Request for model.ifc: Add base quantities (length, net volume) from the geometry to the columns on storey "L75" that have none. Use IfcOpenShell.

First a look at what the model holds.

```python
import ifcopenshell
import ifcopenshell.util.element
import ifcopenshell.util.unit

model = ifcopenshell.open("model.ifc")
print(model.schema)
for unit_type in ("LENGTHUNIT", "AREAUNIT", "VOLUMEUNIT"):
    print(unit_type, ifcopenshell.util.unit.calculate_unit_scale(model, unit_type))
storey = next(s for s in model.by_type("IfcBuildingStorey") if s.Name == "L75")
columns = [e for e in ifcopenshell.util.element.get_decomposition(storey) if e.is_a("IfcColumn")]
for e in sorted(columns, key=lambda e: e.id()):
    print(e.id(), e.is_a(), e.Name, list(ifcopenshell.util.element.get_psets(e, qtos_only=True)), sep=" | ")
```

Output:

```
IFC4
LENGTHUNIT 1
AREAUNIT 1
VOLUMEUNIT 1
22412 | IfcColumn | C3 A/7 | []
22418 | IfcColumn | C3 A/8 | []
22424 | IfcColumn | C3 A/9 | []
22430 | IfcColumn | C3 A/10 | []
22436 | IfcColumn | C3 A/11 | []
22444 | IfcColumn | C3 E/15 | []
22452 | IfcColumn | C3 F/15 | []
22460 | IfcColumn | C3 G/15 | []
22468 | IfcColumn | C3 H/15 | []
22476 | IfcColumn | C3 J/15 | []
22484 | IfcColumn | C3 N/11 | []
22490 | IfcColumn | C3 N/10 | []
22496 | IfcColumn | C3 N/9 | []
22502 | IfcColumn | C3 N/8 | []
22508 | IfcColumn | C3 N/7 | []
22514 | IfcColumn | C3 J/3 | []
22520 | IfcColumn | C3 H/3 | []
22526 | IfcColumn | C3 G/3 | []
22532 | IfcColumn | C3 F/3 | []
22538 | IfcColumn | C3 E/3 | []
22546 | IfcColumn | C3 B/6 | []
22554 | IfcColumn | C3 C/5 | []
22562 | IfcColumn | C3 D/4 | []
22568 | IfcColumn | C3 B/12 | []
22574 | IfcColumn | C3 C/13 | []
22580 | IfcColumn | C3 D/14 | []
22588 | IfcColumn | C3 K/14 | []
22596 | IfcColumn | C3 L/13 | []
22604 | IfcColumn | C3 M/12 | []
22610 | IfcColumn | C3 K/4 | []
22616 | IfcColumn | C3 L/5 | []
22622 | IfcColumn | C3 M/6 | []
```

```python
import ifcopenshell
import ifcopenshell.api.pset
import ifcopenshell.geom
import ifcopenshell.util.element
import ifcopenshell.util.shape
import ifcopenshell.util.unit

model = ifcopenshell.open("model.ifc")
unit_scale = ifcopenshell.util.unit.calculate_unit_scale(model)
volume_scale = ifcopenshell.util.unit.calculate_unit_scale(model, "VOLUMEUNIT")
settings = ifcopenshell.geom.settings()

storey = next(s for s in model.by_type("IfcBuildingStorey") if s.Name == "L75")
columns = [e for e in ifcopenshell.util.element.get_decomposition(storey) if e.is_a("IfcColumn")]

for e in sorted(columns, key=lambda e: e.id()):
    if ifcopenshell.util.element.get_psets(e, qtos_only=True, should_inherit=False):
        continue
    # Geometry comes back in metres, in the element's own axes.
    shape = ifcopenshell.geom.create_shape(settings, e)
    values = {
        "Length": ifcopenshell.util.shape.get_z(shape.geometry) / unit_scale,
        "NetVolume": ifcopenshell.util.shape.get_volume(shape.geometry) / volume_scale,
    }
    qto = ifcopenshell.api.pset.add_qto(model, product=e, name="Qto_ColumnBaseQuantities")
    ifcopenshell.api.pset.edit_qto(model, qto=qto, properties=values)
    print(e.id(), {k: round(v, 3) for k, v in values.items()})

model.write("model_rev.ifc")
```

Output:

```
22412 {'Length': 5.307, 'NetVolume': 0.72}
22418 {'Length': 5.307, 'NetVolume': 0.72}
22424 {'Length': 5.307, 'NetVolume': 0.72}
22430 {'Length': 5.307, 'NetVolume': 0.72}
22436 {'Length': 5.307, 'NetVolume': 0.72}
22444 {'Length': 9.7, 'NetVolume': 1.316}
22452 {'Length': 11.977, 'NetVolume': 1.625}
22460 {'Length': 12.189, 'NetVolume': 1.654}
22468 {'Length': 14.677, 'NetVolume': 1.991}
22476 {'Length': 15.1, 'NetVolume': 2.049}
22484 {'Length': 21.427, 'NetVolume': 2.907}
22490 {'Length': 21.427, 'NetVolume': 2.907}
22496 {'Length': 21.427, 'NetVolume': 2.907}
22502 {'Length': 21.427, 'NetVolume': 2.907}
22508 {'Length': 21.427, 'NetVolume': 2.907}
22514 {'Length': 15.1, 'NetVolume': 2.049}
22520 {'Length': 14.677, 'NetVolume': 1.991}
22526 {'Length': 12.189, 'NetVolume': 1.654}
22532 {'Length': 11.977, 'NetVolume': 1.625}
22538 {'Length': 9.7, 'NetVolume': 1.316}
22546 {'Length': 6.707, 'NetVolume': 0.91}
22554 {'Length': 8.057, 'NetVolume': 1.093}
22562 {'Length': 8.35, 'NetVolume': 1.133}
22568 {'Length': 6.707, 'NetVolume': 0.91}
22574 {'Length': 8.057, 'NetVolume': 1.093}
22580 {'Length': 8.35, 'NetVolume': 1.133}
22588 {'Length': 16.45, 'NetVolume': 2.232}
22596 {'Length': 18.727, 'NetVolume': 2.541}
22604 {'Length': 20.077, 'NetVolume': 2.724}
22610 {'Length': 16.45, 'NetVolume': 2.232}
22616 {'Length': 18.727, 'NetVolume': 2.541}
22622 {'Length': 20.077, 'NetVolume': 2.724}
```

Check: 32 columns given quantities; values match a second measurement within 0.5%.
